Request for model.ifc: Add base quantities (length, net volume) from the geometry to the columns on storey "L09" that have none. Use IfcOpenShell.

First a look at what the model holds.

```python
import ifcopenshell
import ifcopenshell.util.element
import ifcopenshell.util.unit

model = ifcopenshell.open("model.ifc")
print(model.schema)
for unit_type in ("LENGTHUNIT", "AREAUNIT", "VOLUMEUNIT"):
    print(unit_type, ifcopenshell.util.unit.calculate_unit_scale(model, unit_type))
storey = next(s for s in model.by_type("IfcBuildingStorey") if s.Name == "L09")
columns = [e for e in ifcopenshell.util.element.get_decomposition(storey) if e.is_a("IfcColumn")]
for e in sorted(columns, key=lambda e: e.id()):
    print(e.id(), e.is_a(), e.Name, list(ifcopenshell.util.element.get_psets(e, qtos_only=True)), sep=" | ")
```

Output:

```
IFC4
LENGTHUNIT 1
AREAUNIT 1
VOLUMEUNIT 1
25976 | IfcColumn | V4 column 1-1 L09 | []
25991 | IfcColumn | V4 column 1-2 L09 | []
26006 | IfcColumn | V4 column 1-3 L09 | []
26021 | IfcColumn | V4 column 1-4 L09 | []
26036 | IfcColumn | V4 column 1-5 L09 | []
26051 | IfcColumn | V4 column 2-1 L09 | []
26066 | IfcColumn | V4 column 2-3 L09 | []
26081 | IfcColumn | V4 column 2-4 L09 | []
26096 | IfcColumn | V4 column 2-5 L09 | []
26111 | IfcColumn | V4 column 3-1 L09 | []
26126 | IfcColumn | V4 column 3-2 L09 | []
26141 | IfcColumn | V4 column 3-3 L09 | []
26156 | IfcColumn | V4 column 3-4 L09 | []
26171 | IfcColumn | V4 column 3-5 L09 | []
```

```python
import ifcopenshell
import ifcopenshell.api.pset
import ifcopenshell.geom
import ifcopenshell.util.element
import ifcopenshell.util.shape
import ifcopenshell.util.unit

model = ifcopenshell.open("model.ifc")
unit_scale = ifcopenshell.util.unit.calculate_unit_scale(model)
volume_scale = ifcopenshell.util.unit.calculate_unit_scale(model, "VOLUMEUNIT")
settings = ifcopenshell.geom.settings()

storey = next(s for s in model.by_type("IfcBuildingStorey") if s.Name == "L09")
columns = [e for e in ifcopenshell.util.element.get_decomposition(storey) if e.is_a("IfcColumn")]

for e in sorted(columns, key=lambda e: e.id()):
    if ifcopenshell.util.element.get_psets(e, qtos_only=True, should_inherit=False):
        continue
    # Geometry comes back in metres, in the element's own axes.
    shape = ifcopenshell.geom.create_shape(settings, e)
    values = {
        "Length": ifcopenshell.util.shape.get_z(shape.geometry) / unit_scale,
        "NetVolume": ifcopenshell.util.shape.get_volume(shape.geometry) / volume_scale,
    }
    qto = ifcopenshell.api.pset.add_qto(model, product=e, name="Qto_ColumnBaseQuantities")
    ifcopenshell.api.pset.edit_qto(model, qto=qto, properties=values)
    print(e.id(), {k: round(v, 3) for k, v in values.items()})

model.write("model_edited.ifc")
```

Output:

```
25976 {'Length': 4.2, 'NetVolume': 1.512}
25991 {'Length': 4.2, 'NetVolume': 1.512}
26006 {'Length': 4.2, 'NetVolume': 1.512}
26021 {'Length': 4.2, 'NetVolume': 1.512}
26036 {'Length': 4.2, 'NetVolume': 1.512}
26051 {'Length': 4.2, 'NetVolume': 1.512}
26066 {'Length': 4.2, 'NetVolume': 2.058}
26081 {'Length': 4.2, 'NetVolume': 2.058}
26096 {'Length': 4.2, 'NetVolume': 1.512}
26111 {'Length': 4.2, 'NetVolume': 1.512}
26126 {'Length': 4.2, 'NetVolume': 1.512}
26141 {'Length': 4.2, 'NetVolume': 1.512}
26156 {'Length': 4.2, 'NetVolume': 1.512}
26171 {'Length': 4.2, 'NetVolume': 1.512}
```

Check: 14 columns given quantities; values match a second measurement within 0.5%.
